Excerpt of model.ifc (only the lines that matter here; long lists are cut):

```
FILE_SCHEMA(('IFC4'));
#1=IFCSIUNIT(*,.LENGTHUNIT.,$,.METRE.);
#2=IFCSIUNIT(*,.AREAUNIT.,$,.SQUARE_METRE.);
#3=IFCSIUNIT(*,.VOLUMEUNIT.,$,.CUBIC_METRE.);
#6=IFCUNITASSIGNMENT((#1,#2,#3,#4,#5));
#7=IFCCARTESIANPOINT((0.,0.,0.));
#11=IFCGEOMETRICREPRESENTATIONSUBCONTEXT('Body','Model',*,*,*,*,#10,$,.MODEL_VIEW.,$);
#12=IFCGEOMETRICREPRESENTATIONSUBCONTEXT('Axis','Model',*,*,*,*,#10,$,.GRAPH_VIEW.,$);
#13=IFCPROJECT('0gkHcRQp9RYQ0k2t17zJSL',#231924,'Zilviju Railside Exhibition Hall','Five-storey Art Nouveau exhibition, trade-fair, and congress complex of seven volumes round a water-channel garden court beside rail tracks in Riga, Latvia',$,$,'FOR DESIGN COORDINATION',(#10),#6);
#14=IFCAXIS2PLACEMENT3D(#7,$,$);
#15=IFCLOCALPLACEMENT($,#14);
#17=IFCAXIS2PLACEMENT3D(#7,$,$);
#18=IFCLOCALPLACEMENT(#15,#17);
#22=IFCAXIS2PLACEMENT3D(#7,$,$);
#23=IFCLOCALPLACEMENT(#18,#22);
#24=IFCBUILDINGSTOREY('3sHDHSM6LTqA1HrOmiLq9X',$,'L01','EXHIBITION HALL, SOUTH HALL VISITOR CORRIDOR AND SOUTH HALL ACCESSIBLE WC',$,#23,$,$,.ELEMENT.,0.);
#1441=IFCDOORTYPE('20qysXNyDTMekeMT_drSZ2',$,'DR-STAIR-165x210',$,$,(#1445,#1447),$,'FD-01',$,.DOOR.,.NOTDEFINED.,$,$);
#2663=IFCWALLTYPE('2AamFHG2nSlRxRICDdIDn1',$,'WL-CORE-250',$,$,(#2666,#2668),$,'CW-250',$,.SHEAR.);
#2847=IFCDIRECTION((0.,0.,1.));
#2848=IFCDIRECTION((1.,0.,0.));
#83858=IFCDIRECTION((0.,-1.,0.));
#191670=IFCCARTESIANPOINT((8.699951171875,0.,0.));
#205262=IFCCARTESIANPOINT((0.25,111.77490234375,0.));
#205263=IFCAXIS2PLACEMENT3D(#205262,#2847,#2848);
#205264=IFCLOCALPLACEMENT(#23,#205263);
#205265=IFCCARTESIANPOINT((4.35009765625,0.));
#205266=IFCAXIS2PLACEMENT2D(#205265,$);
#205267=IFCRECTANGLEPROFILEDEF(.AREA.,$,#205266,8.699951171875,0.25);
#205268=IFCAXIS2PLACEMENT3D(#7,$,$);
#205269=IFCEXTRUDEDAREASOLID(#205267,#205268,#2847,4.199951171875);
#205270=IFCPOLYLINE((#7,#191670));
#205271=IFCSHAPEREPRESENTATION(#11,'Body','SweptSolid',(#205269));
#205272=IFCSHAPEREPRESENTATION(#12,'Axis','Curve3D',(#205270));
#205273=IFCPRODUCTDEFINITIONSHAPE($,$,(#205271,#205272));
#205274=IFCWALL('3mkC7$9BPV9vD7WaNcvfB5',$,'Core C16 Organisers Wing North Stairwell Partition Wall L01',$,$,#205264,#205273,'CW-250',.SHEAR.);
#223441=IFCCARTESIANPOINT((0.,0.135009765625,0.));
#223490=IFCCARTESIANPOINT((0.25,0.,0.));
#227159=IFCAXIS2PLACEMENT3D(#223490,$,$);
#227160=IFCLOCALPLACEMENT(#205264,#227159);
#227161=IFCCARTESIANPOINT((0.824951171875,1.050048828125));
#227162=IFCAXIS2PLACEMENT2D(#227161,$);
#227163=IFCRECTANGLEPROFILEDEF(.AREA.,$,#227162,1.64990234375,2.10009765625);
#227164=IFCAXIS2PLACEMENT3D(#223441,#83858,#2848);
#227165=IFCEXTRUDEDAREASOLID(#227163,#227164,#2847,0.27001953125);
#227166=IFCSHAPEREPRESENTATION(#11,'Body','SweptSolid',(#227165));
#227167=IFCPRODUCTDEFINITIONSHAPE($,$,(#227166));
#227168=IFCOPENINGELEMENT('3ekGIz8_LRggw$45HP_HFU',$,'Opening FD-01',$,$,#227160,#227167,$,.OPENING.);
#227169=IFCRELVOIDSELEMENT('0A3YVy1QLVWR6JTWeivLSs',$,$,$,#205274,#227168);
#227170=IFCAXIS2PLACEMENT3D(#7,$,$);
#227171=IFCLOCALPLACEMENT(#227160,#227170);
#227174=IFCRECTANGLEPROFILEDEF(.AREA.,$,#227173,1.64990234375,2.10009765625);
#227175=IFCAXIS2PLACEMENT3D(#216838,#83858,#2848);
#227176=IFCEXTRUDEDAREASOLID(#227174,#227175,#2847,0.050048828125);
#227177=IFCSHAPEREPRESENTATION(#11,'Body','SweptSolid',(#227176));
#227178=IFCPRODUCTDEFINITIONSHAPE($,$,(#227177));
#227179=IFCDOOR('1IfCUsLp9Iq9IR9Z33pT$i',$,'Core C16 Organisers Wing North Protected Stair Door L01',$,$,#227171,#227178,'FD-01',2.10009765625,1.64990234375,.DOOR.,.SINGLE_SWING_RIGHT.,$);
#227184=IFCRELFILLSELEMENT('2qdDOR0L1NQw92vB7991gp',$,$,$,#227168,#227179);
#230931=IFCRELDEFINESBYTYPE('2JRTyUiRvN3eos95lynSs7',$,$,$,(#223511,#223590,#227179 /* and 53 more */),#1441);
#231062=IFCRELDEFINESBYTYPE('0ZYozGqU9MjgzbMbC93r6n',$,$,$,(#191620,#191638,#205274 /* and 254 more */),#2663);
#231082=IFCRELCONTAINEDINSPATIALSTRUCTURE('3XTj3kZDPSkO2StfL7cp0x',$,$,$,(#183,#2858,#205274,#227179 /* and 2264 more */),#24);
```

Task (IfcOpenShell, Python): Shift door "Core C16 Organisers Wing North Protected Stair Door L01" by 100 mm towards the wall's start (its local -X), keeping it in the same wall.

```python
import ifcopenshell
import ifcopenshell.api.geometry
import ifcopenshell.util.placement
import ifcopenshell.util.unit

model = ifcopenshell.open("model.ifc")
unit_scale = ifcopenshell.util.unit.calculate_unit_scale(model)

door = model.by_id(227179)
opening = door.FillsVoids[0].RelatingOpeningElement
wall = opening.VoidsElements[0].RelatingBuildingElement

wall_matrix = ifcopenshell.util.placement.get_local_placement(wall.ObjectPlacement)
shift = wall_matrix[:3, 0] * -0.1 / unit_scale
before = ifcopenshell.util.placement.get_local_placement(door.ObjectPlacement)[:3, 3].copy()

# The door is placed relative to its opening, so it follows when the opening moves.
matrix = ifcopenshell.util.placement.get_local_placement(opening.ObjectPlacement)
matrix[:3, 3] += shift
ifcopenshell.api.geometry.edit_object_placement(
    model, product=opening, matrix=matrix, is_si=False, should_transform_children=True
)

after = ifcopenshell.util.placement.get_local_placement(door.ObjectPlacement)[:3, 3]
print("door moved by", (after - before).round(3) + 0.0)

model.write("model_edited.ifc")
```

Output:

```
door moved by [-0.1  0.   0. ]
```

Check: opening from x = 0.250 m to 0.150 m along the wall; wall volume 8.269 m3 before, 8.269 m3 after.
